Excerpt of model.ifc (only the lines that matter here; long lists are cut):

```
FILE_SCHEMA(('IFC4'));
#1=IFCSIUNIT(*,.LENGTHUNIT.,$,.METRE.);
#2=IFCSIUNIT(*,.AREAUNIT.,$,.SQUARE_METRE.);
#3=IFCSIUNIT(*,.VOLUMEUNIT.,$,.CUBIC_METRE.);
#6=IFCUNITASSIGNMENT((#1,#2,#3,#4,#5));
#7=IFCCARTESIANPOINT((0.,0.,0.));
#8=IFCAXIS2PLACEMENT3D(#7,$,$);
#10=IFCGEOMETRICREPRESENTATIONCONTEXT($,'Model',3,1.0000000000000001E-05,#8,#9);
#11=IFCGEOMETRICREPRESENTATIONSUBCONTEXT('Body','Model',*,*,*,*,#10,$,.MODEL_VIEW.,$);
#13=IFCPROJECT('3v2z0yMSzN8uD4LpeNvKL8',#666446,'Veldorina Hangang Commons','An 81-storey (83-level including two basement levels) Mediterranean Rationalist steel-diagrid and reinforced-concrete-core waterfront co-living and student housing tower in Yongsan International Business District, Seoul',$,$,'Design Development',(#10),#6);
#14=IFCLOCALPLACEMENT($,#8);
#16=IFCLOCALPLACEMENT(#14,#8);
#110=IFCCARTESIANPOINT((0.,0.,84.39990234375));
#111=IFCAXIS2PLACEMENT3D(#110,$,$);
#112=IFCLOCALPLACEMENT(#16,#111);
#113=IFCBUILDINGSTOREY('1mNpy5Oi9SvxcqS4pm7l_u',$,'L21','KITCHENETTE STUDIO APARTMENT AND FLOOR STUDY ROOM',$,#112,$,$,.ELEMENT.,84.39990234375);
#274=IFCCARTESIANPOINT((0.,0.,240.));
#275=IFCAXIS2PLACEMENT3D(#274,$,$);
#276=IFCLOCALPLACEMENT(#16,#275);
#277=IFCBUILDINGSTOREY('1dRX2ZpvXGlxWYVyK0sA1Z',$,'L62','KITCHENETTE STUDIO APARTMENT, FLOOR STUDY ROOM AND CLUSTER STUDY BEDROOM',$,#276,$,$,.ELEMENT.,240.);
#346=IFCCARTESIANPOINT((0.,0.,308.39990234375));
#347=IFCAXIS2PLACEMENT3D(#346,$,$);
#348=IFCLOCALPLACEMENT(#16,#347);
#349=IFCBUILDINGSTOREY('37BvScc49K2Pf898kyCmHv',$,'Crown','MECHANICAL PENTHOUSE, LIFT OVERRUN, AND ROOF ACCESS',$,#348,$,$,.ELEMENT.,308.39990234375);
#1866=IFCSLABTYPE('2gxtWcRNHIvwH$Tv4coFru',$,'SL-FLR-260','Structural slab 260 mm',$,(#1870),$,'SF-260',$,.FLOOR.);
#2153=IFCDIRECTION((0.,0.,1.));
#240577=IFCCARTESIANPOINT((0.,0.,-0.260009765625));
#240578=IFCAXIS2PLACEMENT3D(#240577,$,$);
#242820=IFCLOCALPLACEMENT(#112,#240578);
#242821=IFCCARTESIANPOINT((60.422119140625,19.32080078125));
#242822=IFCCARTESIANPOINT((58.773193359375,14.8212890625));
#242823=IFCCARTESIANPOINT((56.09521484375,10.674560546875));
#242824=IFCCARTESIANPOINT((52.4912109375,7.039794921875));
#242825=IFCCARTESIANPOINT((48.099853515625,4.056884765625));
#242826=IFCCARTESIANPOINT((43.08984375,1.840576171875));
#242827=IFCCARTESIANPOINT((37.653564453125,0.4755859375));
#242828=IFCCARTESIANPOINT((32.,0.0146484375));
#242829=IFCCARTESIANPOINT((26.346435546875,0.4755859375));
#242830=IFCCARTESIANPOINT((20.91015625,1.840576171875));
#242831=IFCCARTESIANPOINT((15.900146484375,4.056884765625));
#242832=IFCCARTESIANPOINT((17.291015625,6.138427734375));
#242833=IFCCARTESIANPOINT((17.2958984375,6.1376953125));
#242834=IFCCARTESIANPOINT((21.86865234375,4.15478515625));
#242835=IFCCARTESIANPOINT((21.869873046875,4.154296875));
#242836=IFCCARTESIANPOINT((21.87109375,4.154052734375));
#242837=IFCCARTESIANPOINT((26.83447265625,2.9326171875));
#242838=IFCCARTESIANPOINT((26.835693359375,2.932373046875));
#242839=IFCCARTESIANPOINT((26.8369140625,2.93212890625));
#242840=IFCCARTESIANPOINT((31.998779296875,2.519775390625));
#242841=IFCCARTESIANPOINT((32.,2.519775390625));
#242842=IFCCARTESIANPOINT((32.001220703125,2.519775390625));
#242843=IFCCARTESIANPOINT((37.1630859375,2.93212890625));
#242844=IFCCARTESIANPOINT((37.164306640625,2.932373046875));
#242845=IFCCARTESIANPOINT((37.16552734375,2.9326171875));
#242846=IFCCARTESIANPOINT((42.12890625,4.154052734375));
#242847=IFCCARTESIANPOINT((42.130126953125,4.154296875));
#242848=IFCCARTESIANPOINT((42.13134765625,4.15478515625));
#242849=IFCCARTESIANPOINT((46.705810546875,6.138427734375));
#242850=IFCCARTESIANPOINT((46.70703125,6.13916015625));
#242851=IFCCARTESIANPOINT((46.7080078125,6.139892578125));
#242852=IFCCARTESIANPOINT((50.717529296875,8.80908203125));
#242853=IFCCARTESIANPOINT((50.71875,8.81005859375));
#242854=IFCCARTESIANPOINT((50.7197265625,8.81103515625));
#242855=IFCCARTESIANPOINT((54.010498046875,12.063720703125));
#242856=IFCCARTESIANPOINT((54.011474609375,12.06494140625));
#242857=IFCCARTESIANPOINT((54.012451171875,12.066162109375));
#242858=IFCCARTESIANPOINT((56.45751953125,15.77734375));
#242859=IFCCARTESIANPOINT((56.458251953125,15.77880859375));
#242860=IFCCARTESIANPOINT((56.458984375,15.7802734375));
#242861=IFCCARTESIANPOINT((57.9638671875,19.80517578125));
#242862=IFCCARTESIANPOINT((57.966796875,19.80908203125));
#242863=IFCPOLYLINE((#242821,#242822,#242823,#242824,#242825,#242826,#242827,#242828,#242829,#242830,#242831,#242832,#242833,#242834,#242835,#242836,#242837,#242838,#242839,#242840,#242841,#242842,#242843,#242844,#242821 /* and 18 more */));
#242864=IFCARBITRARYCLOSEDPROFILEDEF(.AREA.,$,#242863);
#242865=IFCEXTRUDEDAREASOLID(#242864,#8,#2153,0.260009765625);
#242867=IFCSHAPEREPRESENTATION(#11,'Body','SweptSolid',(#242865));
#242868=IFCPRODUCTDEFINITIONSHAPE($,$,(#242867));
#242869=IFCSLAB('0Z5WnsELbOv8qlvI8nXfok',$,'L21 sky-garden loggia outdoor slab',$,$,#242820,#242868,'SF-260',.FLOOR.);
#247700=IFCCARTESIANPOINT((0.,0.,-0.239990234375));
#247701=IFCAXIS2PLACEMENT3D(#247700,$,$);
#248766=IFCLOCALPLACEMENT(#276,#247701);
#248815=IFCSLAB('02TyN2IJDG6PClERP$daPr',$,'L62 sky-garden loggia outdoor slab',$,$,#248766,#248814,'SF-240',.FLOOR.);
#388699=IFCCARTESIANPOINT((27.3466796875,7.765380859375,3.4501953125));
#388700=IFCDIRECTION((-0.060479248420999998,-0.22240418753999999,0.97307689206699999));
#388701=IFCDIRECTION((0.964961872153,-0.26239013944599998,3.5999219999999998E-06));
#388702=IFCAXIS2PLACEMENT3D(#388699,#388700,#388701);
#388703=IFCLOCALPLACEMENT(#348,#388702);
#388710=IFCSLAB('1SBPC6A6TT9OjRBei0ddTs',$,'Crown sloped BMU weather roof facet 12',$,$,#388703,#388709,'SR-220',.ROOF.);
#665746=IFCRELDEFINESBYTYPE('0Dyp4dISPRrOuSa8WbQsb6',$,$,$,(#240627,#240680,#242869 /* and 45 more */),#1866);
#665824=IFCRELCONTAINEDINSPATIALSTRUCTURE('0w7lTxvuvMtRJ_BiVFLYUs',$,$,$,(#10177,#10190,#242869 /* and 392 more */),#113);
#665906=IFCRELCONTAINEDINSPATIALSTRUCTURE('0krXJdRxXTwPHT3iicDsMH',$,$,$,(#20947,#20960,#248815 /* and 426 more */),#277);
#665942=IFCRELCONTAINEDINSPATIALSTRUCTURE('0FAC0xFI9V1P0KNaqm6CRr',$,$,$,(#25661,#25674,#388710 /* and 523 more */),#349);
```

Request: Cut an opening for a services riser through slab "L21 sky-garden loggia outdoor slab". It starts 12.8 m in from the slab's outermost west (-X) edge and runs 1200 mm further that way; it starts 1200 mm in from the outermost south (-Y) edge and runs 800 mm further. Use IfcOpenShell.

```python
import numpy as np
import ifcopenshell
import ifcopenshell.api.feature
import ifcopenshell.api.geometry
import ifcopenshell.api.root
import ifcopenshell.geom
import ifcopenshell.util.placement
import ifcopenshell.util.representation
import ifcopenshell.util.shape
import ifcopenshell.util.unit

model = ifcopenshell.open("model.ifc")
unit_scale = ifcopenshell.util.unit.calculate_unit_scale(model)
settings = ifcopenshell.geom.settings()


def volume(element):
    """Net volume in cubic metres, openings subtracted."""
    shape = ifcopenshell.geom.create_shape(settings, element)
    return ifcopenshell.util.shape.get_volume(shape.geometry)


slab = model.by_id(242869)
before = volume(slab)

# Extent in the slab's own axes, in metres. The edges named are its -X and -Y sides.
slab_shape = ifcopenshell.geom.create_shape(settings, slab)
vertices = ifcopenshell.util.shape.get_vertices(slab_shape.geometry)
x_min, y_min, bottom = vertices.min(axis=0)
top = vertices[:, 2].max()

opening = ifcopenshell.api.root.create_entity(model, ifc_class="IfcOpeningElement", name="Services riser opening", predefined_type="OPENING")
context = ifcopenshell.util.representation.get_context(model, "Model", "Body", "MODEL_VIEW")
width, depth = 1.2, 0.8
outline = [(0.0, 0.0), (width, 0.0), (width, depth), (0.0, depth), (0.0, 0.0)]
# Overshoot both faces by 50 mm so the cut is clean.
shape = ifcopenshell.api.geometry.add_slab_representation(
    model, context=context, depth=top - bottom + 0.1, polyline=outline
)
ifcopenshell.api.geometry.assign_representation(model, product=opening, representation=shape)

matrix = ifcopenshell.util.placement.get_local_placement(slab.ObjectPlacement)
matrix[:, 3] = matrix @ np.append(np.array([x_min + 12.8, y_min + 1.2, bottom - 0.05]) / unit_scale, 1.0)
ifcopenshell.api.geometry.edit_object_placement(model, product=opening, matrix=matrix, is_si=False)
ifcopenshell.api.feature.add_feature(model, feature=opening, element=slab)

after = volume(slab)

print(f"slab volume {before:.3f} -> {after:.3f} m3")

model.write("model_updated.ifc")
```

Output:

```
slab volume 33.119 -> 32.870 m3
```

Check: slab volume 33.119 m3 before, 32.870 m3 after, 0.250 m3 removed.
